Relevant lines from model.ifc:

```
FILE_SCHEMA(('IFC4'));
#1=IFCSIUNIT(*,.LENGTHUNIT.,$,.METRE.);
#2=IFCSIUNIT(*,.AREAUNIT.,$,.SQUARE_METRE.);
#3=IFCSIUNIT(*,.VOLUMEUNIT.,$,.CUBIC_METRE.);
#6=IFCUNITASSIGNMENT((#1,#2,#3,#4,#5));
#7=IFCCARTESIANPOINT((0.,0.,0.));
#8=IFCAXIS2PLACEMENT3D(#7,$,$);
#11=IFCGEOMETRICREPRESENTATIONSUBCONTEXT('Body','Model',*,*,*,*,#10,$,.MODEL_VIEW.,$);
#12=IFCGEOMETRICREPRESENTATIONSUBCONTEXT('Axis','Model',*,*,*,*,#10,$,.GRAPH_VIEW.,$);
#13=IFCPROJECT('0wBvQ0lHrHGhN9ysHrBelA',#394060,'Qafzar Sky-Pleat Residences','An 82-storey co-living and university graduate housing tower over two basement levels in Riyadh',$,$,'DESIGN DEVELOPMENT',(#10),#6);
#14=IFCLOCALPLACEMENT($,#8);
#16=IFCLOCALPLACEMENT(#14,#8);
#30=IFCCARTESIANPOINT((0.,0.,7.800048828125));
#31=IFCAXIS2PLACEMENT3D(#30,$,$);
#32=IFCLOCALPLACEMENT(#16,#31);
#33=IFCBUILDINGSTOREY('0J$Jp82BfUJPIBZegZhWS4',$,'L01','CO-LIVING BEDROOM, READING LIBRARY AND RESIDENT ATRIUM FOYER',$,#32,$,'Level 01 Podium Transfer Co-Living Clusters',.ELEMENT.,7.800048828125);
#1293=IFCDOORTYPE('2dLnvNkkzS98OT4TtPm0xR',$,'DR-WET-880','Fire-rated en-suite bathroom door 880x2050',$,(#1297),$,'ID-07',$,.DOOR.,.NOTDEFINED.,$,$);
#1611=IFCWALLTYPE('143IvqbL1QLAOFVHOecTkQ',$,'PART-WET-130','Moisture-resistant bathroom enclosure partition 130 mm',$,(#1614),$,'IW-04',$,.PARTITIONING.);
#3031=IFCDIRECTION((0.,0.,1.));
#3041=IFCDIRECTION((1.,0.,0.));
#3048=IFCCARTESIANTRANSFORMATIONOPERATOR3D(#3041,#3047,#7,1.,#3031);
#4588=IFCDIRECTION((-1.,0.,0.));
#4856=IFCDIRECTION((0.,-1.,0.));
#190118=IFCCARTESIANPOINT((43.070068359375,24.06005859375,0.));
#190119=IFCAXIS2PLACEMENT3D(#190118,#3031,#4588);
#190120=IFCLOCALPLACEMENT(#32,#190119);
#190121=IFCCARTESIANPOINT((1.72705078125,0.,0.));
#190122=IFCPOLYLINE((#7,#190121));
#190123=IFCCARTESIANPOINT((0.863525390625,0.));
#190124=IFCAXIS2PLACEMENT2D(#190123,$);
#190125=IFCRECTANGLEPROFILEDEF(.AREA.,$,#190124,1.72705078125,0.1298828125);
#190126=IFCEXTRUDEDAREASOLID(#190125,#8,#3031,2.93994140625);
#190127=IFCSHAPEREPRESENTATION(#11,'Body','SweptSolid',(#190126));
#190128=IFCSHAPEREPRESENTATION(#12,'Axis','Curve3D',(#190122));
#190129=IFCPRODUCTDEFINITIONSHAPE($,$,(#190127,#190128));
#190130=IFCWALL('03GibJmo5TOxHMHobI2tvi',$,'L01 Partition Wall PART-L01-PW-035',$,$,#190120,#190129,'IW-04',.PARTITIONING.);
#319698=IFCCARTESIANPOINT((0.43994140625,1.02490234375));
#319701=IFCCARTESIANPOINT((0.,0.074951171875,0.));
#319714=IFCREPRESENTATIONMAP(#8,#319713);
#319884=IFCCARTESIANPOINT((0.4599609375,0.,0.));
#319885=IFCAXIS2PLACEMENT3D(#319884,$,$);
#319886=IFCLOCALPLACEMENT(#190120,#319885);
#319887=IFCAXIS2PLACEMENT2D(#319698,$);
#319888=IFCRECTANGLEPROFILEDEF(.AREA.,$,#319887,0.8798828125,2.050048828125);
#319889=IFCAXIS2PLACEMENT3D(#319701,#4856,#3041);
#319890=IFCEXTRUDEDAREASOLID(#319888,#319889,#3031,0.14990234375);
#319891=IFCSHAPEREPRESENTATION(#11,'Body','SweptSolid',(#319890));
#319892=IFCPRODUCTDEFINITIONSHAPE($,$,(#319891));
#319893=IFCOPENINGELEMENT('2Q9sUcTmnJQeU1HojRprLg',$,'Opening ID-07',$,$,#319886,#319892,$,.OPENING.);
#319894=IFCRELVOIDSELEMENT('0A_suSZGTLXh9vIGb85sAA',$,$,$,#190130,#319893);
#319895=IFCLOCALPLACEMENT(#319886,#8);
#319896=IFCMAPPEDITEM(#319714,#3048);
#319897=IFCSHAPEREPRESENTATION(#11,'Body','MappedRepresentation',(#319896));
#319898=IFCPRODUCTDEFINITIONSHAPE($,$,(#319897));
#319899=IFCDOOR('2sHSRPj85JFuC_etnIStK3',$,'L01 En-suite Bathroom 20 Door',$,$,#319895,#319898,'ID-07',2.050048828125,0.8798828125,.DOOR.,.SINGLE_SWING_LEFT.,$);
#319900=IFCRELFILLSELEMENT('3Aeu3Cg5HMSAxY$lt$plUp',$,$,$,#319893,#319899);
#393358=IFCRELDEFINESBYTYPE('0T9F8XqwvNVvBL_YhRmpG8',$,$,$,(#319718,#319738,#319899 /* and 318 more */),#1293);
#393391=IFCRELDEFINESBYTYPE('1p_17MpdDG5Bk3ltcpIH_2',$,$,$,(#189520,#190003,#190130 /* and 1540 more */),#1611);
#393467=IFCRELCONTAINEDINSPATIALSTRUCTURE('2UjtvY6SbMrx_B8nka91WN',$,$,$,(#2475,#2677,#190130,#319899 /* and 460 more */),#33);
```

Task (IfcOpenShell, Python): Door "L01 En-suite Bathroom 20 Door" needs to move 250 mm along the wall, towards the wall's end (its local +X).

```python
import ifcopenshell
import ifcopenshell.api.geometry
import ifcopenshell.util.placement

model = ifcopenshell.open("model.ifc")

door = model.by_guid("2sHSRPj85JFuC_etnIStK3")
opening = door.FillsVoids[0].RelatingOpeningElement
wall = opening.VoidsElements[0].RelatingBuildingElement

wall_matrix = ifcopenshell.util.placement.get_local_placement(wall.ObjectPlacement)
shift = wall_matrix[:3, 0] * 0.25
before = ifcopenshell.util.placement.get_local_placement(door.ObjectPlacement)[:3, 3].copy()

# The door is placed relative to its opening, so it follows when the opening moves.
matrix = ifcopenshell.util.placement.get_local_placement(opening.ObjectPlacement)
matrix[:3, 3] += shift
ifcopenshell.api.geometry.edit_object_placement(
    model, product=opening, matrix=matrix, is_si=False, should_transform_children=True
)

after = ifcopenshell.util.placement.get_local_placement(door.ObjectPlacement)[:3, 3]
print("door moved by", (after - before).round(3) + 0.0)

model.write("model_rev.ifc")
```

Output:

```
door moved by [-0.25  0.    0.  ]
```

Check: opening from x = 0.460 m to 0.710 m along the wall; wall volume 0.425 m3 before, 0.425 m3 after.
